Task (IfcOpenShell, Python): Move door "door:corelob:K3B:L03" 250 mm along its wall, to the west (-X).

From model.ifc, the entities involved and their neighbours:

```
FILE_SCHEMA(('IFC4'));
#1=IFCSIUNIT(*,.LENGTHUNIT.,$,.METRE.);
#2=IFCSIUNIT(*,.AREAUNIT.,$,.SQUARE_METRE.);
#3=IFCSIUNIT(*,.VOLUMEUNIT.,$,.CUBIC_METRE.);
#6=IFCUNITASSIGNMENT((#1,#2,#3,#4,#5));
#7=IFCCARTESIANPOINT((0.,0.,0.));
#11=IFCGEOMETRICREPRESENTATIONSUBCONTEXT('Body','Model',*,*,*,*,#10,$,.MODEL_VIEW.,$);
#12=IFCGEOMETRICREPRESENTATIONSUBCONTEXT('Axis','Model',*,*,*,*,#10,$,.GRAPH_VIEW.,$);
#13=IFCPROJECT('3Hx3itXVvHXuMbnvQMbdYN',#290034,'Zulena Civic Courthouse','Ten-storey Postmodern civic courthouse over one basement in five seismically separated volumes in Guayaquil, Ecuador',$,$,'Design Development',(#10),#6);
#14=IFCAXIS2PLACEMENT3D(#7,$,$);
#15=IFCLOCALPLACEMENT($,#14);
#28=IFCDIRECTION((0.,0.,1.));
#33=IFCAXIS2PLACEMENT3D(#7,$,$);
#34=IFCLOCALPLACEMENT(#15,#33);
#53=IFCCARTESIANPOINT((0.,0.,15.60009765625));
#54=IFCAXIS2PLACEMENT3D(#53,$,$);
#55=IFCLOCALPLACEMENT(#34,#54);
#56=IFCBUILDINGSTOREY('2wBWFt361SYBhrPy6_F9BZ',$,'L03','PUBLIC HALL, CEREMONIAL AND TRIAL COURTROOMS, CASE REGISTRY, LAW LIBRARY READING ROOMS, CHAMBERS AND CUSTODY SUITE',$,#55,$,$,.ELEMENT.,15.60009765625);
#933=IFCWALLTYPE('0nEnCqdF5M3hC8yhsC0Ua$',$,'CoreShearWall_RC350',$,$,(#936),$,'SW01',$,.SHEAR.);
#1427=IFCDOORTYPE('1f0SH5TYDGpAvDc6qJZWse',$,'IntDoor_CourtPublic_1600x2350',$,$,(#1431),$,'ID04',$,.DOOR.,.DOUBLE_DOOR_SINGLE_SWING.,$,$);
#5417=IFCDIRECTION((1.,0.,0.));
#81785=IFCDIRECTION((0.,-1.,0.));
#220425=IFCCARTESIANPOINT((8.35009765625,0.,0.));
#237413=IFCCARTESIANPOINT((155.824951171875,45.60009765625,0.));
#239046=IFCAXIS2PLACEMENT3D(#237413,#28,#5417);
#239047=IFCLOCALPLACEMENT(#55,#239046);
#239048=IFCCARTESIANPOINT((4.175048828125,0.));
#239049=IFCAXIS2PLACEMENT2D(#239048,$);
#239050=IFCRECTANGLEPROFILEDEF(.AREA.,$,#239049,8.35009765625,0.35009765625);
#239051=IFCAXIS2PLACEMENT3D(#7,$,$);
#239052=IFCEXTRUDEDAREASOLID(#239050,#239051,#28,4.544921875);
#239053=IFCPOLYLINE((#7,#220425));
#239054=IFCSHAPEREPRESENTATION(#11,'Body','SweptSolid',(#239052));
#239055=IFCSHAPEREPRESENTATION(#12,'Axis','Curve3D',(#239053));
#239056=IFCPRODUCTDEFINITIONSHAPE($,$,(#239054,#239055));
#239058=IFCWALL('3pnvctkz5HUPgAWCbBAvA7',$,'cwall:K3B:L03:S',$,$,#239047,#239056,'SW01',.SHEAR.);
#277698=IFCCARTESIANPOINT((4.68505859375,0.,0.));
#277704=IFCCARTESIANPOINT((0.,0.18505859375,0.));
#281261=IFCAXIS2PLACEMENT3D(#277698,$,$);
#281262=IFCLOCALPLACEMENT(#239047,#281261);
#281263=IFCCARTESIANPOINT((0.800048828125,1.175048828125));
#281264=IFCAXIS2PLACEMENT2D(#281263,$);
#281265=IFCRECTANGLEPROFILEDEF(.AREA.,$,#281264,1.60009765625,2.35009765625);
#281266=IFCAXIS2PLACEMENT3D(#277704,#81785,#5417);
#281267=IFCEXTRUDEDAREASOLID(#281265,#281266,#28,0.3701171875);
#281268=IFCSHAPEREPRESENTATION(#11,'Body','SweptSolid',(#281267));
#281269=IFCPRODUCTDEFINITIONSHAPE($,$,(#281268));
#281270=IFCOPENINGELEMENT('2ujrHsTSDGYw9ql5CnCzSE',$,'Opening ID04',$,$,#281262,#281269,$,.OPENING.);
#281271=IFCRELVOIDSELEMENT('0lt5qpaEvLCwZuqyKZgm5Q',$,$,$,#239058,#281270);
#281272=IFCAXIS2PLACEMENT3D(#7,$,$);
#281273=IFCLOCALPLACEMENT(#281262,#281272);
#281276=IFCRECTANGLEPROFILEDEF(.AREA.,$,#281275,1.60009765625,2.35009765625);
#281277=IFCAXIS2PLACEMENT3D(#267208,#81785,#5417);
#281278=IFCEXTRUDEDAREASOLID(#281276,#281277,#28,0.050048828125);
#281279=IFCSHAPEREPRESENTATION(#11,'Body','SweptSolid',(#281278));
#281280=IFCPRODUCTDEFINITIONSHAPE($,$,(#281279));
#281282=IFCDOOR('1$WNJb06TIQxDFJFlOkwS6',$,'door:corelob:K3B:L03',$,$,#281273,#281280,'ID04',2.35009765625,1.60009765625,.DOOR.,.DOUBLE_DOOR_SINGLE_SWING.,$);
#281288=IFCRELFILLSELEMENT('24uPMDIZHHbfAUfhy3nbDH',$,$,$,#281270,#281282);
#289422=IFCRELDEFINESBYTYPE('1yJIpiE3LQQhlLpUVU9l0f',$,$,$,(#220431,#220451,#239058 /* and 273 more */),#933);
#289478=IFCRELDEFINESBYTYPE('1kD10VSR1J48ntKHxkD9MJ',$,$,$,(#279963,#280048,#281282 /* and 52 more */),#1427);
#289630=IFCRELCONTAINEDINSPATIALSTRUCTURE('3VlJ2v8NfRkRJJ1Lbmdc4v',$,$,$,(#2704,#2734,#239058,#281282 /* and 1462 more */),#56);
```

```python
import ifcopenshell
import ifcopenshell.api.geometry
import ifcopenshell.util.placement

model = ifcopenshell.open("model.ifc")

door = model.by_guid("1$WNJb06TIQxDFJFlOkwS6")
opening = door.FillsVoids[0].RelatingOpeningElement
wall = opening.VoidsElements[0].RelatingBuildingElement

wall_matrix = ifcopenshell.util.placement.get_local_placement(wall.ObjectPlacement)
shift = wall_matrix[:3, 0] * -0.25
before = ifcopenshell.util.placement.get_local_placement(door.ObjectPlacement)[:3, 3].copy()

# The door is placed relative to its opening, so it follows when the opening moves.
matrix = ifcopenshell.util.placement.get_local_placement(opening.ObjectPlacement)
matrix[:3, 3] += shift
ifcopenshell.api.geometry.edit_object_placement(
    model, product=opening, matrix=matrix, is_si=False, should_transform_children=True
)

after = ifcopenshell.util.placement.get_local_placement(door.ObjectPlacement)[:3, 3]
print("door moved by", (after - before).round(3) + 0.0)

model.write("model_edited.ifc")
```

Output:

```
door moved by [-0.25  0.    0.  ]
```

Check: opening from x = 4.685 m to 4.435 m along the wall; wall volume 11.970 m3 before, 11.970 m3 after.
